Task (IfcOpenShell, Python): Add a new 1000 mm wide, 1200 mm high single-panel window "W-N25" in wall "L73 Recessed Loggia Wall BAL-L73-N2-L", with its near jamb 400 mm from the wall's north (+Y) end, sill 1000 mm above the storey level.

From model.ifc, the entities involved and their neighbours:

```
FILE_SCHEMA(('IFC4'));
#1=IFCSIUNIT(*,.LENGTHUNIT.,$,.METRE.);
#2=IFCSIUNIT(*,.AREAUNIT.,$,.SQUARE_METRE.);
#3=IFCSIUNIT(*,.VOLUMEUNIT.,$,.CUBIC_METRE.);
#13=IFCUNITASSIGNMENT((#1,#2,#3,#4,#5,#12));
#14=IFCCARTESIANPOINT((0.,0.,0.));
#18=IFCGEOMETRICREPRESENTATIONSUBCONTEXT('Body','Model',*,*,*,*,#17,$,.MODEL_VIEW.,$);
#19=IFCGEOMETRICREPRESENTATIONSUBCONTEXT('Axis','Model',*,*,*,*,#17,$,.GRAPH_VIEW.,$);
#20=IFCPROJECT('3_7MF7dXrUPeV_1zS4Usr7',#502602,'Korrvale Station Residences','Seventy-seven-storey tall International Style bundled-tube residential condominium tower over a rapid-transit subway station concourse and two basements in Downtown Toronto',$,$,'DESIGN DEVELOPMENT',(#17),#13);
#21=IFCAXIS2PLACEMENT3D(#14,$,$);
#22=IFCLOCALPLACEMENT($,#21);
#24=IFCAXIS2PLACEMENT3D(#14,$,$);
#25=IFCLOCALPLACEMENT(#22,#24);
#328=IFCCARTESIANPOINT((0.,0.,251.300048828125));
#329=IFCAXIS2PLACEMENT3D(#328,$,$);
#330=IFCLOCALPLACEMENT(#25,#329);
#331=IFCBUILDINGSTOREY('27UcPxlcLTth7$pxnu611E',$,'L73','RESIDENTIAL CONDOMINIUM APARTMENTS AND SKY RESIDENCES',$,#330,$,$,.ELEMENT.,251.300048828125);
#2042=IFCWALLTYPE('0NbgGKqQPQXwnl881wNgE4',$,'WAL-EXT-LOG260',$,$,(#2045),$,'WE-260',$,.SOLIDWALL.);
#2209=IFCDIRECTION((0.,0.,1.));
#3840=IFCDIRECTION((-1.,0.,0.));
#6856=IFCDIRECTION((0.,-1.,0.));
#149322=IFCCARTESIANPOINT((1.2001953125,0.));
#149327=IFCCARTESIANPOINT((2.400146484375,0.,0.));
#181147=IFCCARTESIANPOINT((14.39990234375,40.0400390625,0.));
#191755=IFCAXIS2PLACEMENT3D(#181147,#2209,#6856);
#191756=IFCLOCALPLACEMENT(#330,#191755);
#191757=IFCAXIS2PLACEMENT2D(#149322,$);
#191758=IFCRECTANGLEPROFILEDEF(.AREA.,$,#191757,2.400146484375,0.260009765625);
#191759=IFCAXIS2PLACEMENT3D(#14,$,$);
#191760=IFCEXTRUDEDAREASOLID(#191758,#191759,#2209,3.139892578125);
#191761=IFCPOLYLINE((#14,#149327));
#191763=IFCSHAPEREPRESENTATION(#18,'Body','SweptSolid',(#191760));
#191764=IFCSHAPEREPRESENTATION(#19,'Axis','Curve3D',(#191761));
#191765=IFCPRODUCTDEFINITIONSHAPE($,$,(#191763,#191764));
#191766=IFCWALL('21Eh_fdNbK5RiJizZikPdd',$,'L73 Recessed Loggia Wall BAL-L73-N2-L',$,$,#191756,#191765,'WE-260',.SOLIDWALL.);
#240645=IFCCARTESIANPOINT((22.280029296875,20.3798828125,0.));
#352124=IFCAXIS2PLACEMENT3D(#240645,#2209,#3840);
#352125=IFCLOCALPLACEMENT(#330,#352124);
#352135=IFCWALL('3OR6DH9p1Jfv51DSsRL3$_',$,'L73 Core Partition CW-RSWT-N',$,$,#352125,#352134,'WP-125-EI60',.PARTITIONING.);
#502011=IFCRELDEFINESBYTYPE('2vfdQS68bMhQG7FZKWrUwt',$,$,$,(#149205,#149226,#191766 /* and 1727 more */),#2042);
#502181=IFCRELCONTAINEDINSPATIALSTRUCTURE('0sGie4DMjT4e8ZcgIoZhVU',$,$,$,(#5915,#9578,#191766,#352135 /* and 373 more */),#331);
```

```python
import numpy as np
import ifcopenshell
import ifcopenshell.api.feature
import ifcopenshell.api.geometry
import ifcopenshell.api.root
import ifcopenshell.api.spatial
import ifcopenshell.geom
import ifcopenshell.util.element
import ifcopenshell.util.placement
import ifcopenshell.util.representation
import ifcopenshell.util.shape
import ifcopenshell.util.unit

model = ifcopenshell.open("model.ifc")
unit_scale = ifcopenshell.util.unit.calculate_unit_scale(model)
settings = ifcopenshell.geom.settings()


def volume(element):
    """Net volume in cubic metres, openings subtracted."""
    shape = ifcopenshell.geom.create_shape(settings, element)
    return ifcopenshell.util.shape.get_volume(shape.geometry)


wall = model.by_guid("21Eh_fdNbK5RiJizZikPdd")
storey = ifcopenshell.util.element.get_container(wall, ifc_class="IfcBuildingStorey")
context = ifcopenshell.util.representation.get_context(model, "Model", "Body", "MODEL_VIEW")
before = volume(wall)

width, height, from_end, sill = 1, 1.2, 0.4, 1  # metres

# The wall runs along its own X axis, and the end named is its -X end.
wall_shape = ifcopenshell.geom.create_shape(settings, wall)
x, y, z = ifcopenshell.util.shape.get_vertices(wall_shape.geometry).T
start = x.min() + from_end
face, thickness = float(y.min()), float(y.max() - y.min())
wall_matrix = ifcopenshell.util.placement.get_local_placement(wall.ObjectPlacement)
level = ifcopenshell.util.placement.get_local_placement(storey.ObjectPlacement)[2, 3]


def in_wall(x, y):
    """Placement at x, y metres in the wall's axes, at sill height."""
    matrix = wall_matrix.copy()
    matrix[:, 3] = wall_matrix @ np.array([x / unit_scale, y / unit_scale, 0.0, 1.0])
    matrix[2, 3] = level + sill / unit_scale
    return matrix


# Opening: a box that overshoots both wall faces by 50 mm.
opening = ifcopenshell.api.root.create_entity(model, ifc_class="IfcOpeningElement", predefined_type="OPENING")
box = ifcopenshell.api.geometry.add_wall_representation(
    model, context=context, length=width, height=height, thickness=thickness + 0.1
)
ifcopenshell.api.geometry.assign_representation(model, product=opening, representation=box)
ifcopenshell.api.geometry.edit_object_placement(model, product=opening, matrix=in_wall(start, face - 0.05), is_si=False)
ifcopenshell.api.feature.add_feature(model, feature=opening, element=wall)

window = ifcopenshell.api.root.create_entity(model, ifc_class="IfcWindow", name="W-N25", predefined_type="WINDOW")
window.OverallWidth, window.OverallHeight = width / unit_scale, height / unit_scale
window.PartitioningType = "SINGLE_PANEL"
body = ifcopenshell.api.geometry.add_window_representation(
    model,
    context=context,
    overall_width=window.OverallWidth,
    overall_height=window.OverallHeight,
    partition_type="SINGLE_PANEL",
)
ifcopenshell.api.geometry.assign_representation(model, product=window, representation=body)
ifcopenshell.api.spatial.assign_container(model, products=[window], relating_structure=storey)
ifcopenshell.api.feature.add_filling(model, opening=opening, element=window)

# Centre the window in the wall's thickness.
ifcopenshell.api.geometry.edit_object_placement(model, product=window, matrix=in_wall(start, face), is_si=False)
window_shape = ifcopenshell.geom.create_shape(settings, window)
depth = ifcopenshell.util.shape.get_vertices(window_shape.geometry)[:, 1]
offset = face + thickness / 2 - (depth.min() + depth.max()) / 2
ifcopenshell.api.geometry.edit_object_placement(model, product=window, matrix=in_wall(start, offset), is_si=False)

after = volume(wall)

print(f"wall volume {before:.3f} -> {after:.3f} m3")

model.write("model-out.ifc")
```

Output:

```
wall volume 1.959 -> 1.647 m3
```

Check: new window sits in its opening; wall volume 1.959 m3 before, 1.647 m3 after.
